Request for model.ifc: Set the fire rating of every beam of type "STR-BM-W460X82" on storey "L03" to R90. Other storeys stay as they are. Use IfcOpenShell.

First a look at what the model holds.

```python
import ifcopenshell
import ifcopenshell.util.element

model = ifcopenshell.open("model.ifc")
print(model.schema)
storey = next(s for s in model.by_type("IfcBuildingStorey") if s.Name == "L03")
beams = [e for e in ifcopenshell.util.element.get_decomposition(storey) if e.is_a("IfcBeam")]
seen = {}
for e in beams:
    element_type = ifcopenshell.util.element.get_type(e)
    key = (element_type.Name if element_type != e and element_type else None, ifcopenshell.util.element.get_pset(e, "Pset_BeamCommon", "FireRating"))
    seen[key] = seen.get(key, 0) + 1
for (name, value), count in sorted(seen.items(), key=str):
    print(count, "x", name, "|", value)
```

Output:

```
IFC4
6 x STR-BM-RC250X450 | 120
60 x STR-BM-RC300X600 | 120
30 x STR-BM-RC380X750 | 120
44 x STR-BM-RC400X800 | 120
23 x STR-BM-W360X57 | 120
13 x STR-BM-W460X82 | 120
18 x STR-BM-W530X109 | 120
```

```python
import ifcopenshell
import ifcopenshell.api.pset
import ifcopenshell.util.element

model = ifcopenshell.open("model.ifc")

storey = next(s for s in model.by_type("IfcBuildingStorey") if s.Name == "L03")
beams = [e for e in ifcopenshell.util.element.get_decomposition(storey) if e.is_a("IfcBeam")]

count = 0
for e in beams:
    element_type = ifcopenshell.util.element.get_type(e)
    if element_type in (None, e) or element_type.Name != "STR-BM-W460X82":
        continue
    # add_pset returns the element's existing set when there is one.
    pset = ifcopenshell.api.pset.add_pset(model, product=e, name="Pset_BeamCommon")
    ifcopenshell.api.pset.edit_pset(model, pset=pset, properties={"FireRating": "R90"})
    count += 1

print(count, "beams updated")

model.write("model_rev.ifc")
```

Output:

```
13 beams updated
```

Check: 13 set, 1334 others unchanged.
